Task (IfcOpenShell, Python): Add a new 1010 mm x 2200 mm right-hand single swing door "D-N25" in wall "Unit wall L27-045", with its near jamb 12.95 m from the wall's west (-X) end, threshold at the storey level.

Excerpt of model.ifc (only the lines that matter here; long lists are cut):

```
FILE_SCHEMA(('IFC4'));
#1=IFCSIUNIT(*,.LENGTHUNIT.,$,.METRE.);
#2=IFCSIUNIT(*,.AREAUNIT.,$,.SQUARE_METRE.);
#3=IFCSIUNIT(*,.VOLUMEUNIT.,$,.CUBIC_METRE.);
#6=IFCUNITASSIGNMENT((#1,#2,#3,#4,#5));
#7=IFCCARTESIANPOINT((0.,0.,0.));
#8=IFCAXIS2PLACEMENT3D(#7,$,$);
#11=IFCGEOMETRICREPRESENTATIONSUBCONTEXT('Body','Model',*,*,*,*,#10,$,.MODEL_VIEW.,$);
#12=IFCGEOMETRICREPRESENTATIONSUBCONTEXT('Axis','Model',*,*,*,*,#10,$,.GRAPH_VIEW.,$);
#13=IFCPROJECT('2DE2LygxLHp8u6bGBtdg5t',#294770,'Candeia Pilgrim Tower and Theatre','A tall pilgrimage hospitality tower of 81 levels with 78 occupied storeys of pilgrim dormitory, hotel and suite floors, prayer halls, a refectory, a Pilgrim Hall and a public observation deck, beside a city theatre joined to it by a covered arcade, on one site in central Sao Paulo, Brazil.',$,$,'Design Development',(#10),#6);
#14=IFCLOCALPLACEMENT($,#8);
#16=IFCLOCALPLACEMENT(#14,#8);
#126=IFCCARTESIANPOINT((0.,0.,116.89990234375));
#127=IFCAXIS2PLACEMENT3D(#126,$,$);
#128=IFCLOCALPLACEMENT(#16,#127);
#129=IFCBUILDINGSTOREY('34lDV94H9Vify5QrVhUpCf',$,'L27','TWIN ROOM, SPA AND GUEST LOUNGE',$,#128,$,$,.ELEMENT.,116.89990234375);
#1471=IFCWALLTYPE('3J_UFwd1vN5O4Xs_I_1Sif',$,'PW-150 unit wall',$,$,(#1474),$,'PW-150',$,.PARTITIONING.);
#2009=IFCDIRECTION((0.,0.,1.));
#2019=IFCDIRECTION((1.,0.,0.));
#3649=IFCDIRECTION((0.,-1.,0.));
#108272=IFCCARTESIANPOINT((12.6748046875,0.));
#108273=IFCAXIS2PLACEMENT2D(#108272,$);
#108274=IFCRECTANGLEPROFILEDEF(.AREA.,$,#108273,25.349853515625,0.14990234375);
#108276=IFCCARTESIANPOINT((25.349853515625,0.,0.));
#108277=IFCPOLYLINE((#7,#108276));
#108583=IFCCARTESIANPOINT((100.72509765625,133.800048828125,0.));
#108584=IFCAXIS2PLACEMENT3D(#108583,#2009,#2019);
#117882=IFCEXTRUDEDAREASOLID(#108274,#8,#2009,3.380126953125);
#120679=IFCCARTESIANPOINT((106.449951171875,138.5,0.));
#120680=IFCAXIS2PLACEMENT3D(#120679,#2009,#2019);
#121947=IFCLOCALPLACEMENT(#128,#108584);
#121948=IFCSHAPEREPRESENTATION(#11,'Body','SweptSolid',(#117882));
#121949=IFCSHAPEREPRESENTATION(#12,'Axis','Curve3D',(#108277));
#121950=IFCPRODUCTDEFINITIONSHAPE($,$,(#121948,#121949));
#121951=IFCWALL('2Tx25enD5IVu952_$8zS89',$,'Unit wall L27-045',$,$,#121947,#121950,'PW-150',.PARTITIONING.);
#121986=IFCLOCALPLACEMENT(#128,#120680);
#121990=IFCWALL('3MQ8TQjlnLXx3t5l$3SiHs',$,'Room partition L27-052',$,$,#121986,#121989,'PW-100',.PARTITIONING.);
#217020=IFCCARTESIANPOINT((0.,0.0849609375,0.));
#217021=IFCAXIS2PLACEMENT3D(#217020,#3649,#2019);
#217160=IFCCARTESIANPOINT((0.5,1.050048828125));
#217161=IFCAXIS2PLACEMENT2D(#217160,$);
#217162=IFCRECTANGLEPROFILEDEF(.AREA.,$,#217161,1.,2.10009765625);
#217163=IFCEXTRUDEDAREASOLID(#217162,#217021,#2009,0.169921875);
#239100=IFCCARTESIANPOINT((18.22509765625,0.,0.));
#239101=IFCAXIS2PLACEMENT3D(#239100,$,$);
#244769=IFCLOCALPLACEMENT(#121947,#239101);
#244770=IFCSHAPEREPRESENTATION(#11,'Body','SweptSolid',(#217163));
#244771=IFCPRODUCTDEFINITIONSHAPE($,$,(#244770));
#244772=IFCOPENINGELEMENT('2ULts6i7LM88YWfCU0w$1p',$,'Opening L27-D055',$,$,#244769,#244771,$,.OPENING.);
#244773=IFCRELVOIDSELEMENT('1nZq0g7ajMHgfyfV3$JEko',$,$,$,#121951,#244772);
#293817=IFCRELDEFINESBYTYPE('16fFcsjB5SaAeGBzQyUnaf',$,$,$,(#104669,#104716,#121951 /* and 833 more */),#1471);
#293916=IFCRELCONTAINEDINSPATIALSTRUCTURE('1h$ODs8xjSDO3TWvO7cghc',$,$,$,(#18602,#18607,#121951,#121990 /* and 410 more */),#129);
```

```python
import numpy as np
import ifcopenshell
import ifcopenshell.api.feature
import ifcopenshell.api.geometry
import ifcopenshell.api.root
import ifcopenshell.api.spatial
import ifcopenshell.geom
import ifcopenshell.util.element
import ifcopenshell.util.placement
import ifcopenshell.util.representation
import ifcopenshell.util.shape
import ifcopenshell.util.unit

model = ifcopenshell.open("model.ifc")
unit_scale = ifcopenshell.util.unit.calculate_unit_scale(model)
settings = ifcopenshell.geom.settings()


def volume(element):
    """Net volume in cubic metres, openings subtracted."""
    shape = ifcopenshell.geom.create_shape(settings, element)
    return ifcopenshell.util.shape.get_volume(shape.geometry)


wall = model.by_guid("2Tx25enD5IVu952_$8zS89")
storey = ifcopenshell.util.element.get_container(wall, ifc_class="IfcBuildingStorey")
context = ifcopenshell.util.representation.get_context(model, "Model", "Body", "MODEL_VIEW")
before = volume(wall)

width, height, from_end, sill = 1.01, 2.2, 12.95, 0.0  # metres

# The wall runs along its own X axis, and the end named is its -X end.
wall_shape = ifcopenshell.geom.create_shape(settings, wall)
x, y, z = ifcopenshell.util.shape.get_vertices(wall_shape.geometry).T
start = x.min() + from_end
face, thickness = float(y.min()), float(y.max() - y.min())
wall_matrix = ifcopenshell.util.placement.get_local_placement(wall.ObjectPlacement)
level = ifcopenshell.util.placement.get_local_placement(storey.ObjectPlacement)[2, 3]


def in_wall(x, y):
    """Placement at x, y metres in the wall's axes, at sill height."""
    matrix = wall_matrix.copy()
    matrix[:, 3] = wall_matrix @ np.array([x / unit_scale, y / unit_scale, 0.0, 1.0])
    matrix[2, 3] = level + sill / unit_scale
    return matrix


# Opening: a box that overshoots both wall faces by 50 mm.
opening = ifcopenshell.api.root.create_entity(model, ifc_class="IfcOpeningElement", predefined_type="OPENING")
box = ifcopenshell.api.geometry.add_wall_representation(
    model, context=context, length=width, height=height, thickness=thickness + 0.1
)
ifcopenshell.api.geometry.assign_representation(model, product=opening, representation=box)
ifcopenshell.api.geometry.edit_object_placement(model, product=opening, matrix=in_wall(start, face - 0.05), is_si=False)
ifcopenshell.api.feature.add_feature(model, feature=opening, element=wall)

door = ifcopenshell.api.root.create_entity(model, ifc_class="IfcDoor", name="D-N25", predefined_type="DOOR")
door.OverallWidth, door.OverallHeight = width / unit_scale, height / unit_scale
door.OperationType = "SINGLE_SWING_RIGHT"
body = ifcopenshell.api.geometry.add_door_representation(
    model,
    context=context,
    overall_width=door.OverallWidth,
    overall_height=door.OverallHeight,
    operation_type="SINGLE_SWING_RIGHT",
    lining_properties={"LiningDepth": thickness / unit_scale, "ThresholdDepth": thickness / unit_scale},
)
ifcopenshell.api.geometry.assign_representation(model, product=door, representation=body)
ifcopenshell.api.spatial.assign_container(model, products=[door], relating_structure=storey)
ifcopenshell.api.feature.add_filling(model, opening=opening, element=door)

# The lining spans the wall, so the door starts at the wall face.
ifcopenshell.api.geometry.edit_object_placement(model, product=door, matrix=in_wall(start, face), is_si=False)

after = volume(wall)

print(f"wall volume {before:.3f} -> {after:.3f} m3")

model.write("model_edited.ifc")
```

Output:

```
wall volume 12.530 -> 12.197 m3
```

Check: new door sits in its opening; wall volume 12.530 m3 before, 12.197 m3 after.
